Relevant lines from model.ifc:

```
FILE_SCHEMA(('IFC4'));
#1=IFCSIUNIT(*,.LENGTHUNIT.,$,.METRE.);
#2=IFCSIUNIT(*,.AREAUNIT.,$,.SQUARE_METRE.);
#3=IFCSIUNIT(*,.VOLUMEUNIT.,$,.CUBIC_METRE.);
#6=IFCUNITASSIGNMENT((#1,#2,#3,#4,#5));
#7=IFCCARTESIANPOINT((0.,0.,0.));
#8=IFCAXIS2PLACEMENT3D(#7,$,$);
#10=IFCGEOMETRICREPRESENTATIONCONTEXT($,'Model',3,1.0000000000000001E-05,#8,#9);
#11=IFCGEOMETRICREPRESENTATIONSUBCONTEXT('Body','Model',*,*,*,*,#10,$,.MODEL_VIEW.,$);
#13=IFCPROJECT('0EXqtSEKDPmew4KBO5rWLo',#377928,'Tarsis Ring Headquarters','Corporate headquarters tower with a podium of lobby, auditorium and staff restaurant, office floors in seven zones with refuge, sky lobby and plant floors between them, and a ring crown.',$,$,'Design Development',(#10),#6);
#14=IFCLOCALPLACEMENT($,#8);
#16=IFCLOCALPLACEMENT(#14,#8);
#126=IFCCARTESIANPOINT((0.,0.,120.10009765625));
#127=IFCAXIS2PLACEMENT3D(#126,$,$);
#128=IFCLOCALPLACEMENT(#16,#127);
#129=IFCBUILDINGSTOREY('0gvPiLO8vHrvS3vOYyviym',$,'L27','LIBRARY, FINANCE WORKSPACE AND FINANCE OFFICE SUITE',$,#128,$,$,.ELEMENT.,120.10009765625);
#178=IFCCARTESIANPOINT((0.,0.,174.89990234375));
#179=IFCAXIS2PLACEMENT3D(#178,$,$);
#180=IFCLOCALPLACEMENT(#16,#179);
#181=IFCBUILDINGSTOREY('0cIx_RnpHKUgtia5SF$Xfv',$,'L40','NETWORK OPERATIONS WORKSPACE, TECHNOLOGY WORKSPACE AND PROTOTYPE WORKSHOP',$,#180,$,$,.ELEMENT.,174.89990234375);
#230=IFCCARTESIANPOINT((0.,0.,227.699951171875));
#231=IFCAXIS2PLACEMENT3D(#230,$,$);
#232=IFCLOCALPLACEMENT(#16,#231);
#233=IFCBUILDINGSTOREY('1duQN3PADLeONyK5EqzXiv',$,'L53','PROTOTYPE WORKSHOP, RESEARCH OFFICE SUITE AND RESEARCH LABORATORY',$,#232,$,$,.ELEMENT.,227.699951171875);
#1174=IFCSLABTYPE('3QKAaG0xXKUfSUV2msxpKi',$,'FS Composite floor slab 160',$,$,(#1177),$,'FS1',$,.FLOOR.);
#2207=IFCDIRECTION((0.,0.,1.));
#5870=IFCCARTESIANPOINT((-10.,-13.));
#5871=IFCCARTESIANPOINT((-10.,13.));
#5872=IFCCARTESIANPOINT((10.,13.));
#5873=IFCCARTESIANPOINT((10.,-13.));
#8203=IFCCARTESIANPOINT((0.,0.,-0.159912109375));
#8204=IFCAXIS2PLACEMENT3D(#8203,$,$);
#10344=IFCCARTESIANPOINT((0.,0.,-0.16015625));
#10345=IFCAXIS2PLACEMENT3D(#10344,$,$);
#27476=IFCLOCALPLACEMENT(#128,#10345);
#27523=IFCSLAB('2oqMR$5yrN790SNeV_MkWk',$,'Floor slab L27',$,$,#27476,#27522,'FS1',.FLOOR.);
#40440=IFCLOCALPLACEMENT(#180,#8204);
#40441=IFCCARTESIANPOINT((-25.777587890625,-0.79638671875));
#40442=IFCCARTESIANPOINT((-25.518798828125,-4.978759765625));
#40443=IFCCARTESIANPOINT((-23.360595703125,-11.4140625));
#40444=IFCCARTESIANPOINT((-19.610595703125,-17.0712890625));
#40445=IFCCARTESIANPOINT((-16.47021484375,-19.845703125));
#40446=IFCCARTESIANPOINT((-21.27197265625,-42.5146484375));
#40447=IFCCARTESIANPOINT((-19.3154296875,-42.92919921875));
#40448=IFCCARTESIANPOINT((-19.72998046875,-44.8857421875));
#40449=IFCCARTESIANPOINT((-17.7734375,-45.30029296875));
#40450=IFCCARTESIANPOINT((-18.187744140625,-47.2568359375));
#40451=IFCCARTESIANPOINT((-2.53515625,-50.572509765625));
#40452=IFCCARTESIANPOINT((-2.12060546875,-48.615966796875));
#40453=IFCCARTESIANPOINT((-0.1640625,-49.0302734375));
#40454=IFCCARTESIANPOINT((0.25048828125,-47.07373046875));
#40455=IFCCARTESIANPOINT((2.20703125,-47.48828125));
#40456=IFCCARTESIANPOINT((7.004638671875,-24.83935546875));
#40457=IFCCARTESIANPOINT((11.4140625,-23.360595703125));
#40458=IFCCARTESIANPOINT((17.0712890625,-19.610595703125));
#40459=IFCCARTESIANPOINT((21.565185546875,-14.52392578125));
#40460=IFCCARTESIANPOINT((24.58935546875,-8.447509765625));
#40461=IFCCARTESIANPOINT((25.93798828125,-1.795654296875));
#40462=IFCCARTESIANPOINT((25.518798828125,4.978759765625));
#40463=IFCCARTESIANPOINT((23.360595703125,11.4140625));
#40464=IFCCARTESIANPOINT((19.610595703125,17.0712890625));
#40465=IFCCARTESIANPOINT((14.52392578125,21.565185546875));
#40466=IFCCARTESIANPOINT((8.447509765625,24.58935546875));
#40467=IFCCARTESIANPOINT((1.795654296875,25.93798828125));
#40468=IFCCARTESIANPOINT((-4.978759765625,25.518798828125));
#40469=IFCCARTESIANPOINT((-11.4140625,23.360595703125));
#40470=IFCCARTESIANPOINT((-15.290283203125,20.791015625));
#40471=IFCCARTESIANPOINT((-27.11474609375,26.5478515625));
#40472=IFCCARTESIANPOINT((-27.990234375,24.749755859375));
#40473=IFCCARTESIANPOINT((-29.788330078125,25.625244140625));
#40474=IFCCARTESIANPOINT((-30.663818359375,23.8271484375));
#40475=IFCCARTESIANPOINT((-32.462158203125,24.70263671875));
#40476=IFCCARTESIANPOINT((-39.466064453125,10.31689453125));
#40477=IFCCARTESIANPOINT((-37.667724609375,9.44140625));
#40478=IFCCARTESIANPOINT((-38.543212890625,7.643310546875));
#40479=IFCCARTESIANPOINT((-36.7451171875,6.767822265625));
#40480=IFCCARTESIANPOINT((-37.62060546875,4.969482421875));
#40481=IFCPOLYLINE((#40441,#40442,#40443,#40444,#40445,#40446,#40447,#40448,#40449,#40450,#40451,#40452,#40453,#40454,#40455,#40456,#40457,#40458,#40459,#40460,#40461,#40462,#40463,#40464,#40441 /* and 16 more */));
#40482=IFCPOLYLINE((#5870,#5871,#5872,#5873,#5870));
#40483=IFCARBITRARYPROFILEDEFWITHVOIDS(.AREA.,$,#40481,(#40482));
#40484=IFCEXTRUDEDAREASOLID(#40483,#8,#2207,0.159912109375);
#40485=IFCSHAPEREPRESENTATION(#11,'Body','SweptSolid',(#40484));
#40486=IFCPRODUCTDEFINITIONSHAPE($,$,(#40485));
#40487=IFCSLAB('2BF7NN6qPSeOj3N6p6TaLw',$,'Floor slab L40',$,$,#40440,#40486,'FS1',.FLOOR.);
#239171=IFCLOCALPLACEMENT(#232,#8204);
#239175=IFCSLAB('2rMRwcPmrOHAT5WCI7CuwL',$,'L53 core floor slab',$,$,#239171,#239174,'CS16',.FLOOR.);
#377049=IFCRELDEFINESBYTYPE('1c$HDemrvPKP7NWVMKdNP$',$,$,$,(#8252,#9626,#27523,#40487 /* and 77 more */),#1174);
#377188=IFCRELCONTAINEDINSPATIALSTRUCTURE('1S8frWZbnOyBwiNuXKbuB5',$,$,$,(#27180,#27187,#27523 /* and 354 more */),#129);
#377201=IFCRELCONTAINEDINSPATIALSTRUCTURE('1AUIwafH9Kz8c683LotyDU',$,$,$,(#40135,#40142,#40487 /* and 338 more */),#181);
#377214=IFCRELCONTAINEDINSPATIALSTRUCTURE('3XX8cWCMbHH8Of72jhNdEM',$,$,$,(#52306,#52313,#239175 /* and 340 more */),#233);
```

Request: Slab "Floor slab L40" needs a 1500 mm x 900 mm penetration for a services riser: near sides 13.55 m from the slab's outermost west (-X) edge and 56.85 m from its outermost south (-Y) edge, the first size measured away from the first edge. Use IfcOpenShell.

```python
import numpy as np
import ifcopenshell
import ifcopenshell.api.feature
import ifcopenshell.api.geometry
import ifcopenshell.api.root
import ifcopenshell.geom
import ifcopenshell.util.placement
import ifcopenshell.util.representation
import ifcopenshell.util.shape
import ifcopenshell.util.unit

model = ifcopenshell.open("model.ifc")
unit_scale = ifcopenshell.util.unit.calculate_unit_scale(model)
settings = ifcopenshell.geom.settings()


def volume(element):
    """Net volume in cubic metres, openings subtracted."""
    shape = ifcopenshell.geom.create_shape(settings, element)
    return ifcopenshell.util.shape.get_volume(shape.geometry)


slab = model.by_guid("2BF7NN6qPSeOj3N6p6TaLw")
before = volume(slab)

# Extent in the slab's own axes, in metres. The edges named are its -X and -Y sides.
slab_shape = ifcopenshell.geom.create_shape(settings, slab)
vertices = ifcopenshell.util.shape.get_vertices(slab_shape.geometry)
x_min, y_min, bottom = vertices.min(axis=0)
top = vertices[:, 2].max()

opening = ifcopenshell.api.root.create_entity(model, ifc_class="IfcOpeningElement", name="Services riser opening", predefined_type="OPENING")
context = ifcopenshell.util.representation.get_context(model, "Model", "Body", "MODEL_VIEW")
width, depth = 1.5, 0.9
outline = [(0.0, 0.0), (width, 0.0), (width, depth), (0.0, depth), (0.0, 0.0)]
# Overshoot both faces by 50 mm so the cut is clean.
shape = ifcopenshell.api.geometry.add_slab_representation(
    model, context=context, depth=top - bottom + 0.1, polyline=outline
)
ifcopenshell.api.geometry.assign_representation(model, product=opening, representation=shape)

matrix = ifcopenshell.util.placement.get_local_placement(slab.ObjectPlacement)
matrix[:, 3] = matrix @ np.append(np.array([x_min + 13.55, y_min + 56.85, bottom - 0.05]) / unit_scale, 1.0)
ifcopenshell.api.geometry.edit_object_placement(model, product=opening, matrix=matrix, is_si=False)
ifcopenshell.api.feature.add_feature(model, feature=opening, element=slab)

after = volume(slab)

print(f"slab volume {before:.3f} -> {after:.3f} m3")

model.write("model_rev.ifc")
```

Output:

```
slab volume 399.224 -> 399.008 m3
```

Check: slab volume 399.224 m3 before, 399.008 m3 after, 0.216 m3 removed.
